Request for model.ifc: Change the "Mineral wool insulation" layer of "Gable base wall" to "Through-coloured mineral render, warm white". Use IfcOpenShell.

First a look at what the model holds.

```python
import ifcopenshell
import ifcopenshell.util.element

model = ifcopenshell.open("model.ifc")
print(model.schema)
for layer_set in model.by_type("IfcMaterialLayerSet"):
    if layer_set.LayerSetName == "Gable base wall":
        for layer in layer_set.MaterialLayers:
            print(layer.id(), layer.Material and layer.Material.Name, layer.LayerThickness, sep=" | ")
        print(len(ifcopenshell.util.element.get_elements_by_material(model, layer_set)), "elements and types use it")
print(sorted(m.Name for m in model.by_type("IfcMaterial") if m.Name)[:60])
```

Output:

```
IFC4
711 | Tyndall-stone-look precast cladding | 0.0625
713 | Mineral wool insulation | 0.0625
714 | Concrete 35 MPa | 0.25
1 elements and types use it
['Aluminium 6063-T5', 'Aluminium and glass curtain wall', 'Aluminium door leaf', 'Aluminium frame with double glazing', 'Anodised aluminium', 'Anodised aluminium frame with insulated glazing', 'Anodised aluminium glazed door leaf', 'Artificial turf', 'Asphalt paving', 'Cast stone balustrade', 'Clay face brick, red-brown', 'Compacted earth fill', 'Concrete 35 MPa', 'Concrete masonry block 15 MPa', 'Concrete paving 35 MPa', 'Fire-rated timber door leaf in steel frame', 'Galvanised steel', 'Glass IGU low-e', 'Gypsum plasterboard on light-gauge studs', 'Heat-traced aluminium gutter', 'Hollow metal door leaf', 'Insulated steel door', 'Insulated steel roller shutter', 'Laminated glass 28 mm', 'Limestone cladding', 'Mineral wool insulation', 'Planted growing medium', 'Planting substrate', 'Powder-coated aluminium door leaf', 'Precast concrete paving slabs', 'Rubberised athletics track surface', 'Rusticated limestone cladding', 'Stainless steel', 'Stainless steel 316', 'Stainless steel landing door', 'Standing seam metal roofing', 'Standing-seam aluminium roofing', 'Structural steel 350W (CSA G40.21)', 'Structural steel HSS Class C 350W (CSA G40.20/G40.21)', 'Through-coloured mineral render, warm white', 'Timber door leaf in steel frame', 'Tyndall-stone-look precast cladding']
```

```python
import ifcopenshell
import ifcopenshell.api.material

model = ifcopenshell.open("model.ifc")

layer_set = next(s for s in model.by_type("IfcMaterialLayerSet") if s.LayerSetName == "Gable base wall")
layer = next(l for l in layer_set.MaterialLayers if l.Material and l.Material.Name == "Mineral wool insulation")
material = next(m for m in model.by_type("IfcMaterial") if m.Name == "Through-coloured mineral render, warm white")

# Point this one layer at the other material; renaming the old one would change it everywhere.
ifcopenshell.api.material.edit_layer(model, layer=layer, attributes={"Name": material.Name}, material=material)

print([l.Material.Name if l.Material else None for l in layer_set.MaterialLayers])

model.write("model_rev.ifc")
```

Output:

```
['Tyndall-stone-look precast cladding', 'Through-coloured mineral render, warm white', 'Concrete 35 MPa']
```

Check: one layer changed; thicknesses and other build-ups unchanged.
